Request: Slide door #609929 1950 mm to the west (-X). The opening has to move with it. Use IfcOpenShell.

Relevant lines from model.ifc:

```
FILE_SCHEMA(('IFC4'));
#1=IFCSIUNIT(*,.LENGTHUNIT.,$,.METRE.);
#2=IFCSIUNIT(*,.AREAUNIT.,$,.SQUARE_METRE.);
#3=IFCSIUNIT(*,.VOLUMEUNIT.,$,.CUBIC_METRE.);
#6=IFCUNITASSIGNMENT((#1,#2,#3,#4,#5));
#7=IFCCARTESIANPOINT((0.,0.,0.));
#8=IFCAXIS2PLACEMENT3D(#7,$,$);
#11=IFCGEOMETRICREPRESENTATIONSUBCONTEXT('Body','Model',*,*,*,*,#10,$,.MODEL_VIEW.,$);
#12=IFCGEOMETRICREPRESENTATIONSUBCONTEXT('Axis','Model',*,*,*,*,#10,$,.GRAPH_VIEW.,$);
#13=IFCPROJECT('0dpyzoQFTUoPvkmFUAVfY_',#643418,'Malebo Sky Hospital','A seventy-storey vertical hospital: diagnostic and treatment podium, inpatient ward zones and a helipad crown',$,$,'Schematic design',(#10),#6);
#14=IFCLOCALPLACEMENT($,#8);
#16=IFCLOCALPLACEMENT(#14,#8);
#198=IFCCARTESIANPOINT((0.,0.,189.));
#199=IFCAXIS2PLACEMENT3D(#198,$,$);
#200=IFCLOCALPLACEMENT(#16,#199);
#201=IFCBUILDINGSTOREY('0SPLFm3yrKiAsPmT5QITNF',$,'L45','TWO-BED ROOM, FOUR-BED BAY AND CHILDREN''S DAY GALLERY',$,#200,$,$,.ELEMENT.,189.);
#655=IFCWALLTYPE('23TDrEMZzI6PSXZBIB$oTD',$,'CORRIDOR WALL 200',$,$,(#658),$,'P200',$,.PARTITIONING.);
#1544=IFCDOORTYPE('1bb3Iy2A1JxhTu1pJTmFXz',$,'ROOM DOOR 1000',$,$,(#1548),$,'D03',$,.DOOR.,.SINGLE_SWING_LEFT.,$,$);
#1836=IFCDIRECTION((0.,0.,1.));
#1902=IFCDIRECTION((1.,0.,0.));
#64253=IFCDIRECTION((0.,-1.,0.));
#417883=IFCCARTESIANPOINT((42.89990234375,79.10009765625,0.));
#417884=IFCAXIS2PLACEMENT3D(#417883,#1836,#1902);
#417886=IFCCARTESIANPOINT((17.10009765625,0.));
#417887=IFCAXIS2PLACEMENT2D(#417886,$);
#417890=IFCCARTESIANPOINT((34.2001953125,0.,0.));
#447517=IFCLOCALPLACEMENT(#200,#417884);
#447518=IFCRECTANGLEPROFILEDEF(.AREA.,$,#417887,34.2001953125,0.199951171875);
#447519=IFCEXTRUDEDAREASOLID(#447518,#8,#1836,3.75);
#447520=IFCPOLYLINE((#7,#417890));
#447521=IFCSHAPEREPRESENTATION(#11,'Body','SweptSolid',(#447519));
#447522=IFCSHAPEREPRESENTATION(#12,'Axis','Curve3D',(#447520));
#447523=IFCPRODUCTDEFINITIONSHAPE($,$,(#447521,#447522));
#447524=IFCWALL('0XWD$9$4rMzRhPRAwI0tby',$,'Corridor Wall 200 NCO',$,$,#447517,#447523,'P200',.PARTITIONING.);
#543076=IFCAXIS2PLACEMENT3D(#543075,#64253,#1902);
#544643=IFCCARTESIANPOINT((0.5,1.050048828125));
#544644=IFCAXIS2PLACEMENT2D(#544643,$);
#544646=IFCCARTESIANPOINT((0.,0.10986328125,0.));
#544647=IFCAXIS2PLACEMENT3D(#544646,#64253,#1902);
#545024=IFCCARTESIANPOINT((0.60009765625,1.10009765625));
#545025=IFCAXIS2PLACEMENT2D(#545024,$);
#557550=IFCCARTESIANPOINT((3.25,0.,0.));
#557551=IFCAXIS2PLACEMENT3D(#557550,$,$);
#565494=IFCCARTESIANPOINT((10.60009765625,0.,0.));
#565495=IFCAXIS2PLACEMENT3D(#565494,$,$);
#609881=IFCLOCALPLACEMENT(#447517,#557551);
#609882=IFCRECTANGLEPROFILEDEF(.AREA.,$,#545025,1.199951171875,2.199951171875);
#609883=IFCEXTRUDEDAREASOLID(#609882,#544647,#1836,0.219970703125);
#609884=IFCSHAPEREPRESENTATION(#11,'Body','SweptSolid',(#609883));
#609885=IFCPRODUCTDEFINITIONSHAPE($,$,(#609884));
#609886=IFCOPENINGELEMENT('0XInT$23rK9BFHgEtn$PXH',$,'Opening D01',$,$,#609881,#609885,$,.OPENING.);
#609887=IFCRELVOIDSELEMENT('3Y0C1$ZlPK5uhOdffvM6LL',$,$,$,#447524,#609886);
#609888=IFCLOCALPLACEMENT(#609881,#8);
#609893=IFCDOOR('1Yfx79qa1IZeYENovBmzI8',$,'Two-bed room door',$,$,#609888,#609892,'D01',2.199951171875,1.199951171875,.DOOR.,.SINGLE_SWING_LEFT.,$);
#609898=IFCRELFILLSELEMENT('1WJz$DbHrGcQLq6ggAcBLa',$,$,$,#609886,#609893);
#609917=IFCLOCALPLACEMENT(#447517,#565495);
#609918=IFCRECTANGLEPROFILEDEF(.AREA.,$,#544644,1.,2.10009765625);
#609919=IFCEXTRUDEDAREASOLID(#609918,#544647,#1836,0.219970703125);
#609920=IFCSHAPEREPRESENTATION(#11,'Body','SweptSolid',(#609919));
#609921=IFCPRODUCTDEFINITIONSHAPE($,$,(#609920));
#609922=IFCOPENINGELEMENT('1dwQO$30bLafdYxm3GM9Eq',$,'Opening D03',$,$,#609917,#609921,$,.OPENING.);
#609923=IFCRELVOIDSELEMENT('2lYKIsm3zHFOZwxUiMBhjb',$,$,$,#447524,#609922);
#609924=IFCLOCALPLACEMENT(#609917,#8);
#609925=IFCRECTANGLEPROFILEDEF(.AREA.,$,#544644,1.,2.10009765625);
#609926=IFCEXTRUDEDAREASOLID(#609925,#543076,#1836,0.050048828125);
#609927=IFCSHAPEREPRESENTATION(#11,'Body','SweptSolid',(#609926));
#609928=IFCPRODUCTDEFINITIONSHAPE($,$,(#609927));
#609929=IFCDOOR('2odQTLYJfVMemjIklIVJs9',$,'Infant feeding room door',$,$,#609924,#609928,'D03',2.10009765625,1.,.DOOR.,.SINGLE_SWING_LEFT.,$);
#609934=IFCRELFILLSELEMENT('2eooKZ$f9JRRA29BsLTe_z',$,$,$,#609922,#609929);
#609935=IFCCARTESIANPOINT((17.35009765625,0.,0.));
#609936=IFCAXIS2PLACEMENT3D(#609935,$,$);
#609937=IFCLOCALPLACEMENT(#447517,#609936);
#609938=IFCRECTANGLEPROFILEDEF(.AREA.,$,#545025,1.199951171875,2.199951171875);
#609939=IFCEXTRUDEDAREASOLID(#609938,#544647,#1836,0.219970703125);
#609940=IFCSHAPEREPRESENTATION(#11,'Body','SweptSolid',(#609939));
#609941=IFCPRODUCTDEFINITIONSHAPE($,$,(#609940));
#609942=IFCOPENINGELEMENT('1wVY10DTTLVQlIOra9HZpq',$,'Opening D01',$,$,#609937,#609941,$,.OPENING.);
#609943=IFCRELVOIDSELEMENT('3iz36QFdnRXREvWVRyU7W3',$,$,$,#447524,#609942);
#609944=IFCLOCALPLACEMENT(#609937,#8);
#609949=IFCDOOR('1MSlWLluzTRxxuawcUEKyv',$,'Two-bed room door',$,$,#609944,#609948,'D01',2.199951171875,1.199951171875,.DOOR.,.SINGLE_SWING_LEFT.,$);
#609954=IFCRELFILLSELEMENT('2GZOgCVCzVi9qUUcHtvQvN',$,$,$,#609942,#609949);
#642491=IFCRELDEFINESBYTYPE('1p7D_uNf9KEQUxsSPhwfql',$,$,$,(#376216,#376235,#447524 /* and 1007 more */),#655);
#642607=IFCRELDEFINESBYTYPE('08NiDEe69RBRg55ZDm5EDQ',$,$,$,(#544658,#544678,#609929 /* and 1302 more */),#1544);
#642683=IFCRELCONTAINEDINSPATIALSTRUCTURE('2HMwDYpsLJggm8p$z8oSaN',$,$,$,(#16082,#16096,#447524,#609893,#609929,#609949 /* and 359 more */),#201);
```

```python
import ifcopenshell
import ifcopenshell.api.geometry
import ifcopenshell.util.placement

model = ifcopenshell.open("model.ifc")

door = model.by_id(609929)
opening = door.FillsVoids[0].RelatingOpeningElement
wall = opening.VoidsElements[0].RelatingBuildingElement

wall_matrix = ifcopenshell.util.placement.get_local_placement(wall.ObjectPlacement)
shift = wall_matrix[:3, 0] * -1.95
before = ifcopenshell.util.placement.get_local_placement(door.ObjectPlacement)[:3, 3].copy()

# The door is placed relative to its opening, so it follows when the opening moves.
matrix = ifcopenshell.util.placement.get_local_placement(opening.ObjectPlacement)
matrix[:3, 3] += shift
ifcopenshell.api.geometry.edit_object_placement(
    model, product=opening, matrix=matrix, is_si=False, should_transform_children=True
)

after = ifcopenshell.util.placement.get_local_placement(door.ObjectPlacement)[:3, 3]
print("door moved by", (after - before).round(3) + 0.0)

model.write("model-out.ifc")
```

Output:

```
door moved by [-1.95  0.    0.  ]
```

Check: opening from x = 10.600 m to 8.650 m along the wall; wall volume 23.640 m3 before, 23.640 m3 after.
